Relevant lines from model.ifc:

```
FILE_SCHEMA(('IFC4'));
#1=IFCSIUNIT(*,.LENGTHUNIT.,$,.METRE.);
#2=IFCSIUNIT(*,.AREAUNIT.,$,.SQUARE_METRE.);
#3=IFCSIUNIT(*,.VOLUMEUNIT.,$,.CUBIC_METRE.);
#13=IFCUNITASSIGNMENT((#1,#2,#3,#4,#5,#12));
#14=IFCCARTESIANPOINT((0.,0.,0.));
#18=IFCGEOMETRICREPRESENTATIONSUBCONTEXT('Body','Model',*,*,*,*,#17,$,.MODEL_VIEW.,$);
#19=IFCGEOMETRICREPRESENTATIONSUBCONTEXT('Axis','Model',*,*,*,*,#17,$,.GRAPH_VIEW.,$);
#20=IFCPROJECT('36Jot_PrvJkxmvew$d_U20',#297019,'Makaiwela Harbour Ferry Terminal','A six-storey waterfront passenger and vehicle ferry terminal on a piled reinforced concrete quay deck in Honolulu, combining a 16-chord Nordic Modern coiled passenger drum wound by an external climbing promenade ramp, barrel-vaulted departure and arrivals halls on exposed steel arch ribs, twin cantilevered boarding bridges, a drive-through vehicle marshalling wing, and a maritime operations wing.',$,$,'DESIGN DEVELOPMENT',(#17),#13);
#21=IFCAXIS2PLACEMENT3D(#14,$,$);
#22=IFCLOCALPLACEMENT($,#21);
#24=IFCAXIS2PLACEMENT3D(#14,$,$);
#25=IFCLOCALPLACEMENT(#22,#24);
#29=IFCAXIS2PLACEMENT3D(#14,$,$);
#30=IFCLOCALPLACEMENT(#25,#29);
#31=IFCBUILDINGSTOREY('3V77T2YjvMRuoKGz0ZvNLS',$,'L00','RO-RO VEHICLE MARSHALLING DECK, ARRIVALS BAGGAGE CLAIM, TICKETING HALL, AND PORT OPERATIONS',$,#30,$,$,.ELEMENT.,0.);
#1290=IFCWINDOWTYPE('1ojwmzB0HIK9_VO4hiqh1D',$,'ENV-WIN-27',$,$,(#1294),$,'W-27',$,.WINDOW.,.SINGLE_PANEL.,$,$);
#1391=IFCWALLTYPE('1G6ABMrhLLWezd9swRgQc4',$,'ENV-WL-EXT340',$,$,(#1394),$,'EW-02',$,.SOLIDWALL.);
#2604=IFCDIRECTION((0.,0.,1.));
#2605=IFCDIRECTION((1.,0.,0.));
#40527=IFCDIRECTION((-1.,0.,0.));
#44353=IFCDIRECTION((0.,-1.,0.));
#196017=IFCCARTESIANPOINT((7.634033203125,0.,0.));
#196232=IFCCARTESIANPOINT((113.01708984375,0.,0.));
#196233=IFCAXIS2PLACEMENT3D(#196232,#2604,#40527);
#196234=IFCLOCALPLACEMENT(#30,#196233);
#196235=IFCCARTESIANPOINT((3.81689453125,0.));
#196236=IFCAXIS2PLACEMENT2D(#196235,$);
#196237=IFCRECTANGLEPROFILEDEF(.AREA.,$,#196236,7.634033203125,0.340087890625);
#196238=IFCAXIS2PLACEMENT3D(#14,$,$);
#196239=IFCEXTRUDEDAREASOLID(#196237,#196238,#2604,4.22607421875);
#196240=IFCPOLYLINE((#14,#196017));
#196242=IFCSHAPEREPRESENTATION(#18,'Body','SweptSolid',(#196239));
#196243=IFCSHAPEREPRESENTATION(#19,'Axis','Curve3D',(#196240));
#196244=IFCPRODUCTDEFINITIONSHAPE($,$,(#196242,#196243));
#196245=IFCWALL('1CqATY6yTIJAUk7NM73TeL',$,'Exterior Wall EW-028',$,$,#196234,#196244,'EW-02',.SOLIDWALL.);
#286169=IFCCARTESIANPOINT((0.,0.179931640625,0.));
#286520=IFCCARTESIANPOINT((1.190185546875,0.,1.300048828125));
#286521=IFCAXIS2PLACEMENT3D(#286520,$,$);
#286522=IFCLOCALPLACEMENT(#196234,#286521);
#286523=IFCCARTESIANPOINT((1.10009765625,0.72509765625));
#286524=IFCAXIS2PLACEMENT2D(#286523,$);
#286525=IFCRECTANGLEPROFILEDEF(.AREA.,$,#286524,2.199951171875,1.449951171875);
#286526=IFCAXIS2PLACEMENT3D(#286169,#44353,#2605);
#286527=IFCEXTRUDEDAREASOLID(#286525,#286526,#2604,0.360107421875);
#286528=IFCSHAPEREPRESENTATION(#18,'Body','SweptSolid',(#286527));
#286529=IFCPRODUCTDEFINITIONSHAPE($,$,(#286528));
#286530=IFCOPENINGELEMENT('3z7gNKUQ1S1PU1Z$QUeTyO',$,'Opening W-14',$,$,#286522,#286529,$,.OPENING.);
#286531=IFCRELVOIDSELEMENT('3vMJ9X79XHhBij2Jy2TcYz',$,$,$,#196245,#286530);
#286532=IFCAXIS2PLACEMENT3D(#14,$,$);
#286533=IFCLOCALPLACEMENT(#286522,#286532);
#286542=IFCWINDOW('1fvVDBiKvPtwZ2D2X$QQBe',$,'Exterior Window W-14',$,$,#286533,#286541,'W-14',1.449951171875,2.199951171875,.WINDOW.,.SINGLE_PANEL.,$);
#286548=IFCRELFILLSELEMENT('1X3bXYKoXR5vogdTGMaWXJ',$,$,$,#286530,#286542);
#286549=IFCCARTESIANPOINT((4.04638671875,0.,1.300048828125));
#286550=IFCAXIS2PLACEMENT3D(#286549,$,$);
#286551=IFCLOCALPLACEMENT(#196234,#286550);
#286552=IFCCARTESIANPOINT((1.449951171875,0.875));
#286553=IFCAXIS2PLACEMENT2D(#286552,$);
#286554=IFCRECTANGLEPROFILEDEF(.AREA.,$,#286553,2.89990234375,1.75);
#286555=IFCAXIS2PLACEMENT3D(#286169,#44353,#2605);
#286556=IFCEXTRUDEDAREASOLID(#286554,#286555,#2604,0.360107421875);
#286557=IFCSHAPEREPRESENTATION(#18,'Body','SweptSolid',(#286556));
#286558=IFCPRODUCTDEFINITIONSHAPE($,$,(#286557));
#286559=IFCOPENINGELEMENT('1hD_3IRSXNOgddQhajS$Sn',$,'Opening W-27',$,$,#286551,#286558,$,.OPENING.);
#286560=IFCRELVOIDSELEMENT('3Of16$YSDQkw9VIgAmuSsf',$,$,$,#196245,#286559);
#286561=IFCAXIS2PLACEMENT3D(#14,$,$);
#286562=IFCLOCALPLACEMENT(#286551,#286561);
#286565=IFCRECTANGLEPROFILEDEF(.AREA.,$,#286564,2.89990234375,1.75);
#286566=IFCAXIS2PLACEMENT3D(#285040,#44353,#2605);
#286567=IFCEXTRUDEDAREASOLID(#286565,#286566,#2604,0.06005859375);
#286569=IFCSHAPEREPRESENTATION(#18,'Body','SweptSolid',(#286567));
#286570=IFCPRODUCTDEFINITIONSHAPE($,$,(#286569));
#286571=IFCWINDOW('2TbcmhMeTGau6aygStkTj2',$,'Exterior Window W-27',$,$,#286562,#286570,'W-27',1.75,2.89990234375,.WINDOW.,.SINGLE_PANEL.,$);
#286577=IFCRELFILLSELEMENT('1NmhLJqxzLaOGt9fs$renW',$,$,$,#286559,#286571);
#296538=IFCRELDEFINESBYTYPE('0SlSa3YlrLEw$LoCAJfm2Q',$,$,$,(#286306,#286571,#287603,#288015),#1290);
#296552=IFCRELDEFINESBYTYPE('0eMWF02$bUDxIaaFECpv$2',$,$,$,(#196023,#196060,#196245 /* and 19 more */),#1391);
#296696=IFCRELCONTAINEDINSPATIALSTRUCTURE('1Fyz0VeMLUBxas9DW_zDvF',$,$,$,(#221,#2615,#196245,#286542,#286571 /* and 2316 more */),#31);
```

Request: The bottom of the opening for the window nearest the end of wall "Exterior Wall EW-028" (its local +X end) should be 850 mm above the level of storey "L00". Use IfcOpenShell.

```python
import numpy as np
import ifcopenshell
import ifcopenshell.api.geometry
import ifcopenshell.geom
import ifcopenshell.util.element
import ifcopenshell.util.placement
import ifcopenshell.util.shape
import ifcopenshell.util.unit

model = ifcopenshell.open("model.ifc")
unit_scale = ifcopenshell.util.unit.calculate_unit_scale(model)

window = model.by_id(286571)
opening = window.FillsVoids[0].RelatingOpeningElement
storey = ifcopenshell.util.element.get_container(window, ifc_class="IfcBuildingStorey")
level = ifcopenshell.util.placement.get_local_placement(storey.ObjectPlacement)[2, 3]

# The opening's origin need not be at the sill, so measure its lowest point.
shape = ifcopenshell.geom.create_shape(ifcopenshell.geom.settings(), opening)
bottom = ifcopenshell.util.shape.get_shape_bottom_elevation(shape, shape.geometry) / unit_scale
dz = level + 0.85 - bottom

shift = np.array([0.0, 0.0, dz])
# The window is placed relative to its opening, so it follows when the opening moves.
matrix = ifcopenshell.util.placement.get_local_placement(opening.ObjectPlacement)
matrix[:3, 3] += shift
ifcopenshell.api.geometry.edit_object_placement(
    model, product=opening, matrix=matrix, is_si=False, should_transform_children=True
)

print(f"moved by {dz * unit_scale:+.3f} m")

model.write("model_rev.ifc")
```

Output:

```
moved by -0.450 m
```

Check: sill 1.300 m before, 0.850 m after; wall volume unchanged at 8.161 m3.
